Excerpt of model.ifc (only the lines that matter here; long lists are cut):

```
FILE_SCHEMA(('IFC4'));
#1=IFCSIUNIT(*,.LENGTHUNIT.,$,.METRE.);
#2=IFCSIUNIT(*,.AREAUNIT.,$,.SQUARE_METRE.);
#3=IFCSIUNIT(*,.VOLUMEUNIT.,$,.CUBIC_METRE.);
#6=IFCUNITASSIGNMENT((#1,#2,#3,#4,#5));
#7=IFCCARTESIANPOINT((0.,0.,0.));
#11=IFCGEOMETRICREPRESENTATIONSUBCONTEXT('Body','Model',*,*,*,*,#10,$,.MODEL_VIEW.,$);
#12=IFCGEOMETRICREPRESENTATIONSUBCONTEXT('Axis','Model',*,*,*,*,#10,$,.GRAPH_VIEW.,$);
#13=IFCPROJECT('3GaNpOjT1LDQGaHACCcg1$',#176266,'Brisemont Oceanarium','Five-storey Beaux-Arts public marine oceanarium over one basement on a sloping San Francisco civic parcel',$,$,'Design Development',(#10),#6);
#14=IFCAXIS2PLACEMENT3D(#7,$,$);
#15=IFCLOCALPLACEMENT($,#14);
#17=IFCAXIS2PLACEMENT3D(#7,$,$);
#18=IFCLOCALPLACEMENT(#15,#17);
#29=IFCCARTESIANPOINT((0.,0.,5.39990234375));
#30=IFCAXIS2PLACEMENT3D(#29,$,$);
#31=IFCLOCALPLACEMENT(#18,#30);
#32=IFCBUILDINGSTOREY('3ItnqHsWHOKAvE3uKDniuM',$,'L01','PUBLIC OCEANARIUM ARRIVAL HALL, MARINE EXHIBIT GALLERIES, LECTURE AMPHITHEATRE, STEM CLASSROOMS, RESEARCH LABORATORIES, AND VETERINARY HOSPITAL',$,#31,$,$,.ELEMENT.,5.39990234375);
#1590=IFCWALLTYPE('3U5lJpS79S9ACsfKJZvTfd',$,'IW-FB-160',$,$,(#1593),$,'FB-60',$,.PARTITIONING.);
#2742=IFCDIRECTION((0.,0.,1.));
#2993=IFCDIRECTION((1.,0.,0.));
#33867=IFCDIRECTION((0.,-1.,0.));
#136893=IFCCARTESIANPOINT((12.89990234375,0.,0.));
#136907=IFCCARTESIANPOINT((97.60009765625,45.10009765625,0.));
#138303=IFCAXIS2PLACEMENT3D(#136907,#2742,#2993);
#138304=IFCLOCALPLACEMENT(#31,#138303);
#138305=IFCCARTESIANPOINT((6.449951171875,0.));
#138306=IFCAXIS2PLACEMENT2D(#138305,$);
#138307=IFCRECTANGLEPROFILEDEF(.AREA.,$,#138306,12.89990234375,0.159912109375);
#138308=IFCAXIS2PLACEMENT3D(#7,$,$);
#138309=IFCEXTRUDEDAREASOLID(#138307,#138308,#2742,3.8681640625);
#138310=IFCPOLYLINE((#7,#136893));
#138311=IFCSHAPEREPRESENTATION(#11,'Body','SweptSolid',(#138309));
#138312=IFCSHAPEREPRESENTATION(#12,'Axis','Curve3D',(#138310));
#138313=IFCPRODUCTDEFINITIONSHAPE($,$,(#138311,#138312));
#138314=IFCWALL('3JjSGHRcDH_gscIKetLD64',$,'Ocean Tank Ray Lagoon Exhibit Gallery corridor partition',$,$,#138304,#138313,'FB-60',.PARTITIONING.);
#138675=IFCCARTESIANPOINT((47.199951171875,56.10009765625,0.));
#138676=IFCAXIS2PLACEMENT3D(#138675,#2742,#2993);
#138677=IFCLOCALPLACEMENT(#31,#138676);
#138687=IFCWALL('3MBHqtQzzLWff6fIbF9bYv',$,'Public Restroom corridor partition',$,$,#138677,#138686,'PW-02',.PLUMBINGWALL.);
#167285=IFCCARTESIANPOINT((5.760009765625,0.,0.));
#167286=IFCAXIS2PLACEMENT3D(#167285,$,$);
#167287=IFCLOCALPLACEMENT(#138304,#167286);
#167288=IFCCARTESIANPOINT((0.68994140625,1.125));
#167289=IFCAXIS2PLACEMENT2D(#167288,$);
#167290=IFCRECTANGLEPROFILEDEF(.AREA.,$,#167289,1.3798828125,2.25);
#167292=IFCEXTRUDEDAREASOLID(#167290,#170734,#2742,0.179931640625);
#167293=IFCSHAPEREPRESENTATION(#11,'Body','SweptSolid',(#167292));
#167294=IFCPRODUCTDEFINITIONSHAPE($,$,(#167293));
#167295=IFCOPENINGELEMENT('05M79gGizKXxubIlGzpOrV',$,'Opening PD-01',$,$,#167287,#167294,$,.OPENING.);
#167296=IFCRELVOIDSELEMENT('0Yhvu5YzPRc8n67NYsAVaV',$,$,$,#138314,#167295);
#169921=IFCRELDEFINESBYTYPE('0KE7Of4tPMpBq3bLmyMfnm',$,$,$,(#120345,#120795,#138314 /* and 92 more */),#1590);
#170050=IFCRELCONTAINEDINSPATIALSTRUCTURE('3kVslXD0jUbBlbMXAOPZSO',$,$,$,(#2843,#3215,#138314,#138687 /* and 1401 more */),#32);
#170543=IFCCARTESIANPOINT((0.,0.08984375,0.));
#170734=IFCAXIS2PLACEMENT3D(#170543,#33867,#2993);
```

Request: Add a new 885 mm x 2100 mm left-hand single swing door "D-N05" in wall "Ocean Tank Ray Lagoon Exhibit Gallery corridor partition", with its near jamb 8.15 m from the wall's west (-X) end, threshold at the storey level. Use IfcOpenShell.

```python
import numpy as np
import ifcopenshell
import ifcopenshell.api.feature
import ifcopenshell.api.geometry
import ifcopenshell.api.root
import ifcopenshell.api.spatial
import ifcopenshell.geom
import ifcopenshell.util.element
import ifcopenshell.util.placement
import ifcopenshell.util.representation
import ifcopenshell.util.shape
import ifcopenshell.util.unit

model = ifcopenshell.open("model.ifc")
unit_scale = ifcopenshell.util.unit.calculate_unit_scale(model)
settings = ifcopenshell.geom.settings()


def volume(element):
    """Net volume in cubic metres, openings subtracted."""
    shape = ifcopenshell.geom.create_shape(settings, element)
    return ifcopenshell.util.shape.get_volume(shape.geometry)


wall = model.by_guid("3JjSGHRcDH_gscIKetLD64")
storey = ifcopenshell.util.element.get_container(wall, ifc_class="IfcBuildingStorey")
context = ifcopenshell.util.representation.get_context(model, "Model", "Body", "MODEL_VIEW")
before = volume(wall)

width, height, from_end, sill = 0.885, 2.1, 8.15, 0.0  # metres

# The wall runs along its own X axis, and the end named is its -X end.
wall_shape = ifcopenshell.geom.create_shape(settings, wall)
x, y, z = ifcopenshell.util.shape.get_vertices(wall_shape.geometry).T
start = x.min() + from_end
face, thickness = float(y.min()), float(y.max() - y.min())
wall_matrix = ifcopenshell.util.placement.get_local_placement(wall.ObjectPlacement)
level = ifcopenshell.util.placement.get_local_placement(storey.ObjectPlacement)[2, 3]


def in_wall(x, y):
    """Placement at x, y metres in the wall's axes, at sill height."""
    matrix = wall_matrix.copy()
    matrix[:, 3] = wall_matrix @ np.array([x / unit_scale, y / unit_scale, 0.0, 1.0])
    matrix[2, 3] = level + sill / unit_scale
    return matrix


# Opening: a box that overshoots both wall faces by 50 mm.
opening = ifcopenshell.api.root.create_entity(model, ifc_class="IfcOpeningElement", predefined_type="OPENING")
box = ifcopenshell.api.geometry.add_wall_representation(
    model, context=context, length=width, height=height, thickness=thickness + 0.1
)
ifcopenshell.api.geometry.assign_representation(model, product=opening, representation=box)
ifcopenshell.api.geometry.edit_object_placement(model, product=opening, matrix=in_wall(start, face - 0.05), is_si=False)
ifcopenshell.api.feature.add_feature(model, feature=opening, element=wall)

door = ifcopenshell.api.root.create_entity(model, ifc_class="IfcDoor", name="D-N05", predefined_type="DOOR")
door.OverallWidth, door.OverallHeight = width / unit_scale, height / unit_scale
door.OperationType = "SINGLE_SWING_LEFT"
body = ifcopenshell.api.geometry.add_door_representation(
    model,
    context=context,
    overall_width=door.OverallWidth,
    overall_height=door.OverallHeight,
    operation_type="SINGLE_SWING_LEFT",
    lining_properties={"LiningDepth": thickness / unit_scale, "ThresholdDepth": thickness / unit_scale},
)
ifcopenshell.api.geometry.assign_representation(model, product=door, representation=body)
ifcopenshell.api.spatial.assign_container(model, products=[door], relating_structure=storey)
ifcopenshell.api.feature.add_filling(model, opening=opening, element=door)

# The lining spans the wall, so the door starts at the wall face.
ifcopenshell.api.geometry.edit_object_placement(model, product=door, matrix=in_wall(start, face), is_si=False)

after = volume(wall)

print(f"wall volume {before:.3f} -> {after:.3f} m3")

model.write("model-out.ifc")
```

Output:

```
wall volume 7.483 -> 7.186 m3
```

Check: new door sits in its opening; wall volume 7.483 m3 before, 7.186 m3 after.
